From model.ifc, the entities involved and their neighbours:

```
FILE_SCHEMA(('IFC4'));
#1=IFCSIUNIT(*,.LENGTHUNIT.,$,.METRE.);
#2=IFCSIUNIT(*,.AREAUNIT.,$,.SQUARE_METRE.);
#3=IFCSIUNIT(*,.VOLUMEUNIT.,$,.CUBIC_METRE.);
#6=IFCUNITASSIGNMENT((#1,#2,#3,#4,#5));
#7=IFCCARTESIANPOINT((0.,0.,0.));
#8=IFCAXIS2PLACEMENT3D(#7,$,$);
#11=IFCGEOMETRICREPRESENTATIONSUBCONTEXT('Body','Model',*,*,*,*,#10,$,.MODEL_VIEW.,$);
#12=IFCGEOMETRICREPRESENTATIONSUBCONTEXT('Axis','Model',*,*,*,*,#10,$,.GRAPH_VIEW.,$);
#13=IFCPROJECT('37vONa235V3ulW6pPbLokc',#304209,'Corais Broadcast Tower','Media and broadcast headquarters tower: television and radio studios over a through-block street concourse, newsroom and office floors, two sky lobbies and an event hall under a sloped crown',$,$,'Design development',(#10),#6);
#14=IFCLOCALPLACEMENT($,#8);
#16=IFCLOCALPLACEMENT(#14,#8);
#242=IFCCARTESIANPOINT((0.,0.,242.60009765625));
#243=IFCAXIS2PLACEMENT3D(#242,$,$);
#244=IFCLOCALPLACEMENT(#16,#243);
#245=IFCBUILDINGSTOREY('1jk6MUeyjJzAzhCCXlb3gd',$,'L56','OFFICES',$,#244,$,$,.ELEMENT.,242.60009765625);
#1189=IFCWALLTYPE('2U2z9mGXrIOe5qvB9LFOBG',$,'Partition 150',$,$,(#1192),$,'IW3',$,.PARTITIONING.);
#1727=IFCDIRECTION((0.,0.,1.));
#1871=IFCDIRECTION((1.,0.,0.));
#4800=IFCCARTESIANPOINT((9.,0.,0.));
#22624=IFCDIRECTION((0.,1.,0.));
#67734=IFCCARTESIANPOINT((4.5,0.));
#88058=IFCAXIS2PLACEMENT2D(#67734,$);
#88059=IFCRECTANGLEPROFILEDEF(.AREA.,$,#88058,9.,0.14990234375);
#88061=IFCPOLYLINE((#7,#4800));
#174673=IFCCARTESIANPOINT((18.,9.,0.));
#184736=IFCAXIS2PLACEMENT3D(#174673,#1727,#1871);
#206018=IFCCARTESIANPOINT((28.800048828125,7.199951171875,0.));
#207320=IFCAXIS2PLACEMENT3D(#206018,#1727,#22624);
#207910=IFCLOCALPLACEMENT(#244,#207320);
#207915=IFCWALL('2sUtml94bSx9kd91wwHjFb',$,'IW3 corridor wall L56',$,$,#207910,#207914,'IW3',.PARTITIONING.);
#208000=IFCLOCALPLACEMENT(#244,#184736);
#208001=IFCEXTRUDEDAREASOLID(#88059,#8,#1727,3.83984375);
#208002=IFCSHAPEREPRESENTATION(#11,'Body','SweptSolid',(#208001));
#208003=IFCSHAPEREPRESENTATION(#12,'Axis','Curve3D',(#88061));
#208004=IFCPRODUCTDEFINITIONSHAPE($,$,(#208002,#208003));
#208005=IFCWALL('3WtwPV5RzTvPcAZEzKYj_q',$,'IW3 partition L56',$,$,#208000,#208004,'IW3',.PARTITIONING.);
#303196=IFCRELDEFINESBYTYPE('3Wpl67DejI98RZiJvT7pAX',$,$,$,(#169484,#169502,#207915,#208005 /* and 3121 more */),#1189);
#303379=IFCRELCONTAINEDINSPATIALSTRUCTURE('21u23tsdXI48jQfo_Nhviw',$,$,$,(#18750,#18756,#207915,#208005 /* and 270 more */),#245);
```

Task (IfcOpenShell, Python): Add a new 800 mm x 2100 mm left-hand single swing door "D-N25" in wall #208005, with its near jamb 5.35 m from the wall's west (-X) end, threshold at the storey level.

```python
import numpy as np
import ifcopenshell
import ifcopenshell.api.feature
import ifcopenshell.api.geometry
import ifcopenshell.api.root
import ifcopenshell.api.spatial
import ifcopenshell.geom
import ifcopenshell.util.element
import ifcopenshell.util.placement
import ifcopenshell.util.representation
import ifcopenshell.util.shape
import ifcopenshell.util.unit

model = ifcopenshell.open("model.ifc")
unit_scale = ifcopenshell.util.unit.calculate_unit_scale(model)
settings = ifcopenshell.geom.settings()


def volume(element):
    """Net volume in cubic metres, openings subtracted."""
    shape = ifcopenshell.geom.create_shape(settings, element)
    return ifcopenshell.util.shape.get_volume(shape.geometry)


wall = model.by_guid("3WtwPV5RzTvPcAZEzKYj_q")
storey = ifcopenshell.util.element.get_container(wall, ifc_class="IfcBuildingStorey")
context = ifcopenshell.util.representation.get_context(model, "Model", "Body", "MODEL_VIEW")
before = volume(wall)

width, height, from_end, sill = 0.8, 2.1, 5.35, 0.0  # metres

# The wall runs along its own X axis, and the end named is its -X end.
wall_shape = ifcopenshell.geom.create_shape(settings, wall)
x, y, z = ifcopenshell.util.shape.get_vertices(wall_shape.geometry).T
start = x.min() + from_end
face, thickness = float(y.min()), float(y.max() - y.min())
wall_matrix = ifcopenshell.util.placement.get_local_placement(wall.ObjectPlacement)
level = ifcopenshell.util.placement.get_local_placement(storey.ObjectPlacement)[2, 3]


def in_wall(x, y):
    """Placement at x, y metres in the wall's axes, at sill height."""
    matrix = wall_matrix.copy()
    matrix[:, 3] = wall_matrix @ np.array([x / unit_scale, y / unit_scale, 0.0, 1.0])
    matrix[2, 3] = level + sill / unit_scale
    return matrix


# Opening: a box that overshoots both wall faces by 50 mm.
opening = ifcopenshell.api.root.create_entity(model, ifc_class="IfcOpeningElement", predefined_type="OPENING")
box = ifcopenshell.api.geometry.add_wall_representation(
    model, context=context, length=width, height=height, thickness=thickness + 0.1
)
ifcopenshell.api.geometry.assign_representation(model, product=opening, representation=box)
ifcopenshell.api.geometry.edit_object_placement(model, product=opening, matrix=in_wall(start, face - 0.05), is_si=False)
ifcopenshell.api.feature.add_feature(model, feature=opening, element=wall)

door = ifcopenshell.api.root.create_entity(model, ifc_class="IfcDoor", name="D-N25", predefined_type="DOOR")
door.OverallWidth, door.OverallHeight = width / unit_scale, height / unit_scale
door.OperationType = "SINGLE_SWING_LEFT"
body = ifcopenshell.api.geometry.add_door_representation(
    model,
    context=context,
    overall_width=door.OverallWidth,
    overall_height=door.OverallHeight,
    operation_type="SINGLE_SWING_LEFT",
    lining_properties={"LiningDepth": thickness / unit_scale, "ThresholdDepth": thickness / unit_scale},
)
ifcopenshell.api.geometry.assign_representation(model, product=door, representation=body)
ifcopenshell.api.spatial.assign_container(model, products=[door], relating_structure=storey)
ifcopenshell.api.feature.add_filling(model, opening=opening, element=door)

# The lining spans the wall, so the door starts at the wall face.
ifcopenshell.api.geometry.edit_object_placement(model, product=door, matrix=in_wall(start, face), is_si=False)

after = volume(wall)

print(f"wall volume {before:.3f} -> {after:.3f} m3")

model.write("model-out.ifc")
```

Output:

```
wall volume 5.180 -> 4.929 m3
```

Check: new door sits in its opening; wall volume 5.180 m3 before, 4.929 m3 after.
